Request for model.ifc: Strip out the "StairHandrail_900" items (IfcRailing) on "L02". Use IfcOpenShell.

First a look at what the model holds.

```python
import ifcopenshell
import ifcopenshell.util.element

model = ifcopenshell.open("model.ifc")
print(model.schema)
storey = next(s for s in model.by_type("IfcBuildingStorey") if s.Name == "L02")
railings = [e for e in ifcopenshell.util.element.get_decomposition(storey) if e.is_a("IfcRailing")]
seen = {}
for e in railings:
    element_type = ifcopenshell.util.element.get_type(e)
    name = element_type.Name if element_type not in (None, e) else None
    seen[name] = seen.get(name, 0) + 1
for name, count in sorted(seen.items(), key=str):
    print(count, "x", name)
```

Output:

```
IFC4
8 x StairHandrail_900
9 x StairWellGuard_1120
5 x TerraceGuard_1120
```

```python
import ifcopenshell
import ifcopenshell.api.root
import ifcopenshell.util.element

model = ifcopenshell.open("model.ifc")

storey = next(s for s in model.by_type("IfcBuildingStorey") if s.Name == "L02")
railings = [e for e in ifcopenshell.util.element.get_decomposition(storey) if e.is_a("IfcRailing")]
targets = [e for e in railings if (t := ifcopenshell.util.element.get_type(e)) not in (None, e) and t.Name == "StairHandrail_900"]

for e in targets:
    ifcopenshell.api.root.remove_product(model, product=e)
print(len(targets), "removed")

model.write("model_edited.ifc")
```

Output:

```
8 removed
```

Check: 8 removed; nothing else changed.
